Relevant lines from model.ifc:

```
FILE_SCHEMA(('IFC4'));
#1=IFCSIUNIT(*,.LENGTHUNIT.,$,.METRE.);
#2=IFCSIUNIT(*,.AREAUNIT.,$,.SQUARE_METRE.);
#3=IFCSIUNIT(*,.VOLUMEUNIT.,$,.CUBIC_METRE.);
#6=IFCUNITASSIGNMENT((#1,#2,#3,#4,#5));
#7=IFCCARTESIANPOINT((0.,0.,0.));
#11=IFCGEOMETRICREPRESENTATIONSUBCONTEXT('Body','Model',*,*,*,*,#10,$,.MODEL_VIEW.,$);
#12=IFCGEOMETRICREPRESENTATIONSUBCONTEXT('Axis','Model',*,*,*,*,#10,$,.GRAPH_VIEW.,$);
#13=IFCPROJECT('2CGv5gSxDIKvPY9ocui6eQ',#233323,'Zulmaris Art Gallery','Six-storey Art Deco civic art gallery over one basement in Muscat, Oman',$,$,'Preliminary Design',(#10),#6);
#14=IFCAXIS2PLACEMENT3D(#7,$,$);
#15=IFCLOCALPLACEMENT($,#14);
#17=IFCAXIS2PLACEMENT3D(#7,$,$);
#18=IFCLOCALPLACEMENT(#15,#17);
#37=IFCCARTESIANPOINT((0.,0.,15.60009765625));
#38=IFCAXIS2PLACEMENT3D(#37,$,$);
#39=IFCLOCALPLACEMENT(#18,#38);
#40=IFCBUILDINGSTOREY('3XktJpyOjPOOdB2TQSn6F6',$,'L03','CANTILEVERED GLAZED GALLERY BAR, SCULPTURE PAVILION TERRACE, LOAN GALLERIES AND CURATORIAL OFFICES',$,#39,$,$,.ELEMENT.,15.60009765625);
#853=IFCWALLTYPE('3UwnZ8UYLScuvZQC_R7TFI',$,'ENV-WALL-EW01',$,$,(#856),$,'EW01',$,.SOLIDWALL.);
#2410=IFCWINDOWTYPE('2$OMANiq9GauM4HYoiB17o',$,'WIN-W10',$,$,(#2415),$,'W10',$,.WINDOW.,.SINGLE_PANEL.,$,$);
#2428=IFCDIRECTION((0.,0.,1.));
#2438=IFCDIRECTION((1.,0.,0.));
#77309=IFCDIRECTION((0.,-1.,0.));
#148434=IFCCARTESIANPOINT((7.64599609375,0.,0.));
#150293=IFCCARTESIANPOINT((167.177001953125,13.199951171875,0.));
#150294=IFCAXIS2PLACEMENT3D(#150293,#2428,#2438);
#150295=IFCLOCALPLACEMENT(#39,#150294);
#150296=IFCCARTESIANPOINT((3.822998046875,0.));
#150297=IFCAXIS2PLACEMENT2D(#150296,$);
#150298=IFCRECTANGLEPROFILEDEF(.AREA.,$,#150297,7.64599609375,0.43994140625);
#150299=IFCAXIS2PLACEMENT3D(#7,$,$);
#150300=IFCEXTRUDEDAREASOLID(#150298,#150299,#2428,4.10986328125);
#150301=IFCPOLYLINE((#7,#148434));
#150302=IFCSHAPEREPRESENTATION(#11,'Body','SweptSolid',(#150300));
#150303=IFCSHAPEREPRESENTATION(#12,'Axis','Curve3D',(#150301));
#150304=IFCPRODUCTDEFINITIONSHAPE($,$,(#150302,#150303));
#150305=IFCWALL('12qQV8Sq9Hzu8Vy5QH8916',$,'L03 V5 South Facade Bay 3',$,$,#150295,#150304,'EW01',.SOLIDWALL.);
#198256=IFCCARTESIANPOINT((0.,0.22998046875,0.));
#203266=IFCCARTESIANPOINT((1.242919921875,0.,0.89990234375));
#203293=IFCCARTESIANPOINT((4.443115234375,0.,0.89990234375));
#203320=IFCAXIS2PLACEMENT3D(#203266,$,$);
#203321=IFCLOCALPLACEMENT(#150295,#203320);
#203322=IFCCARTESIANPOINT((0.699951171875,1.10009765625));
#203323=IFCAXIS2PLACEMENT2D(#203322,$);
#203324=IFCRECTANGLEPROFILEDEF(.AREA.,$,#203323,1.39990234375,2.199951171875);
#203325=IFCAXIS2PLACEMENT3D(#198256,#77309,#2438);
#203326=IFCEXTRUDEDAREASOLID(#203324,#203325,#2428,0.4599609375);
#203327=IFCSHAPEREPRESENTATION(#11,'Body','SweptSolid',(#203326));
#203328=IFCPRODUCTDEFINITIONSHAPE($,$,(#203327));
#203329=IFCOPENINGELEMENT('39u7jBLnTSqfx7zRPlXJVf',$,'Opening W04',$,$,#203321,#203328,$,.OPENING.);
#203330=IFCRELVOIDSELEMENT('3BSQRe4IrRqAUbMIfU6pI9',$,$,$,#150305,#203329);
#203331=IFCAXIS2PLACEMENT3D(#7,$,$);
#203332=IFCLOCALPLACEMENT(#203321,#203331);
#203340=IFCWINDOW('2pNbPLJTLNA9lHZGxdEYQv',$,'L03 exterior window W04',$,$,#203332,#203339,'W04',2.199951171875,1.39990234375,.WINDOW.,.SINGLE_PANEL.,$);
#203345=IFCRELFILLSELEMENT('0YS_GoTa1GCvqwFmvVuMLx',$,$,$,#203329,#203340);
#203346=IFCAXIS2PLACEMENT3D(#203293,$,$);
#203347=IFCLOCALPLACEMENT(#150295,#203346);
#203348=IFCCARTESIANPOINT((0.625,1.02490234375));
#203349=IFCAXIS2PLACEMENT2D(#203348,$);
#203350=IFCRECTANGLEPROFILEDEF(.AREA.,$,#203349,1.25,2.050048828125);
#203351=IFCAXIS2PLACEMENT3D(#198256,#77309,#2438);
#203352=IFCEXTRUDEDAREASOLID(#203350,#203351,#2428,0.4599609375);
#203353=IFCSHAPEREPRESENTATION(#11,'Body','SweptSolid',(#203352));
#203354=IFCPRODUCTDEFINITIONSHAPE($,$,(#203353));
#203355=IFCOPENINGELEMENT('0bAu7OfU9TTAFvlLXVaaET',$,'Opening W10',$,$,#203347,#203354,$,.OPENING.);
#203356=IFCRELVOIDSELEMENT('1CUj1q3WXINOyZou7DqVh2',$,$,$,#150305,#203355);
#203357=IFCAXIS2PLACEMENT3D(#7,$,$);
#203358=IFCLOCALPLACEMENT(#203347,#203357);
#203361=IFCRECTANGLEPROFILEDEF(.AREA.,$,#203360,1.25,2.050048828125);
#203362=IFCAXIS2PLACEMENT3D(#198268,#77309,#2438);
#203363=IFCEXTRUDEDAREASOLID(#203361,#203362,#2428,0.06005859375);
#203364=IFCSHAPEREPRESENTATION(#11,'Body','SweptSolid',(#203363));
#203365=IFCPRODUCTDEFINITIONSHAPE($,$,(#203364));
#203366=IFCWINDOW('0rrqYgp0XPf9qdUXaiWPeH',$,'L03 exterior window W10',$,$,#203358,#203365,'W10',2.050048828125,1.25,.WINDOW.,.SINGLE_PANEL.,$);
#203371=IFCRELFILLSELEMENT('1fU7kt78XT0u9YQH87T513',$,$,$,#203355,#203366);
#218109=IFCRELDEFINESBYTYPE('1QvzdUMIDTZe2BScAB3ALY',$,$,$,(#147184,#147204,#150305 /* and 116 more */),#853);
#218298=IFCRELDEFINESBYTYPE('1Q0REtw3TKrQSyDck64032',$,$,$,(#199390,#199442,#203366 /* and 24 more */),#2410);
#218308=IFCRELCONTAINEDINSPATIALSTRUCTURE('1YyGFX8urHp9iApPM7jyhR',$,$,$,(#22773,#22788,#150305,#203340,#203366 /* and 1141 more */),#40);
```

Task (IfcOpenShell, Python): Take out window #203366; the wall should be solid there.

```python
import ifcopenshell
import ifcopenshell.api.feature
import ifcopenshell.api.root
import ifcopenshell.geom
import ifcopenshell.util.shape

model = ifcopenshell.open("model.ifc")
settings = ifcopenshell.geom.settings()


def volume(element):
    """Net volume in cubic metres, openings subtracted."""
    shape = ifcopenshell.geom.create_shape(settings, element)
    return ifcopenshell.util.shape.get_volume(shape.geometry)


window = model.by_id(203366)
opening = window.FillsVoids[0].RelatingOpeningElement
wall = opening.VoidsElements[0].RelatingBuildingElement
before = volume(wall)

ifcopenshell.api.root.remove_product(model, product=window)
ifcopenshell.api.feature.remove_feature(model, feature=opening)

after = volume(wall)

print(f"wall volume {before:.3f} -> {after:.3f} m3")

model.write("model_edited.ifc")
```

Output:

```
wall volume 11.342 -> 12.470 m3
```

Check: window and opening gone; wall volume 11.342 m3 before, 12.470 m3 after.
